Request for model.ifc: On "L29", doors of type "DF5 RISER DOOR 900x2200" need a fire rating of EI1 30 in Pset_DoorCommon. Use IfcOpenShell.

First a look at what the model holds.

```python
import ifcopenshell
import ifcopenshell.util.element

model = ifcopenshell.open("model.ifc")
print(model.schema)
storey = next(s for s in model.by_type("IfcBuildingStorey") if s.Name == "L29")
doors = [e for e in ifcopenshell.util.element.get_decomposition(storey) if e.is_a("IfcDoor")]
seen = {}
for e in doors:
    element_type = ifcopenshell.util.element.get_type(e)
    key = (element_type.Name if element_type != e and element_type else None, ifcopenshell.util.element.get_pset(e, "Pset_DoorCommon", "FireRating"))
    seen[key] = seen.get(key, 0) + 1
for (name, value), count in sorted(seen.items(), key=str):
    print(count, "x", name, "|", value)
```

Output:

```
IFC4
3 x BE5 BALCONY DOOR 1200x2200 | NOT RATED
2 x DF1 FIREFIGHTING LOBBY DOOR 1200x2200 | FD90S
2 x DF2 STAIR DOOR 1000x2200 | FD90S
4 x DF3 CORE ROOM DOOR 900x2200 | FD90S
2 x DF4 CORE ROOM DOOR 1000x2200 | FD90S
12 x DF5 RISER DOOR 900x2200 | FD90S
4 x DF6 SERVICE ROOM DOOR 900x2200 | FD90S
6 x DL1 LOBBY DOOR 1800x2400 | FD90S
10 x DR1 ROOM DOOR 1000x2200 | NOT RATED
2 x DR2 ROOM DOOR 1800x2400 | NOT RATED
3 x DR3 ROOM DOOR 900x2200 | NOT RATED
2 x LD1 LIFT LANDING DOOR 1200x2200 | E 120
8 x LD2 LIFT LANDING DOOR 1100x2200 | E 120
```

```python
import ifcopenshell
import ifcopenshell.api.pset
import ifcopenshell.util.element

model = ifcopenshell.open("model.ifc")

storey = next(s for s in model.by_type("IfcBuildingStorey") if s.Name == "L29")
doors = [e for e in ifcopenshell.util.element.get_decomposition(storey) if e.is_a("IfcDoor")]

count = 0
for e in doors:
    element_type = ifcopenshell.util.element.get_type(e)
    if element_type in (None, e) or element_type.Name != "DF5 RISER DOOR 900x2200":
        continue
    found = ifcopenshell.util.element.get_pset(e, "Pset_DoorCommon", should_inherit=False)
    if found:
        pset = model.by_id(found["id"])
        if len(ifcopenshell.util.element.get_elements_by_pset(pset)) > 1:
            pset = ifcopenshell.api.pset.unshare_pset(model, products=[e], pset=pset)[0]
    else:
        pset = ifcopenshell.api.pset.add_pset(model, product=e, name="Pset_DoorCommon")
    ifcopenshell.api.pset.edit_pset(model, pset=pset, properties={"FireRating": "EI1 30"})
    count += 1

print(count, "doors updated")

model.write("model_updated.ifc")
```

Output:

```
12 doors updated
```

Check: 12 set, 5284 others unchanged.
